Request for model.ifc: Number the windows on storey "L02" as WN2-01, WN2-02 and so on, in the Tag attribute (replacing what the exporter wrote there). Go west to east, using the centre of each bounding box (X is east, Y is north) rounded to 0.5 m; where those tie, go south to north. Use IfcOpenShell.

First a look at what the model holds.

```python
import ifcopenshell
import ifcopenshell.util.element
import ifcopenshell.util.placement

model = ifcopenshell.open("model.ifc")
print(model.schema)
storey = next(s for s in model.by_type("IfcBuildingStorey") if s.Name == "L02")
windows = [e for e in ifcopenshell.util.element.get_decomposition(storey) if e.is_a("IfcWindow")]
for e in sorted(windows, key=lambda e: e.id()):
    origin = ifcopenshell.util.placement.get_local_placement(e.ObjectPlacement)[:3, 3]
    print(e.id(), e.Tag, e.Name, origin.round(2) + 0.0, sep=" | ")
```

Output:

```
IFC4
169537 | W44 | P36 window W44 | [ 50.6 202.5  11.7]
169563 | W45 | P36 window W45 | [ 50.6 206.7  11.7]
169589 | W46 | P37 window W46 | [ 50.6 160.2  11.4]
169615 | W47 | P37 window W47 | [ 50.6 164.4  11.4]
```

```python
import ifcopenshell
import ifcopenshell.geom
import ifcopenshell.util.element
import ifcopenshell.util.shape

model = ifcopenshell.open("model.ifc")
settings = ifcopenshell.geom.settings()
settings.set("use-world-coords", True)


def centre(element):
    shape = ifcopenshell.geom.create_shape(settings, element)
    return ifcopenshell.util.shape.get_bbox_centroid(shape.geometry)


storey = next(s for s in model.by_type("IfcBuildingStorey") if s.Name == "L02")
windows = [e for e in ifcopenshell.util.element.get_decomposition(storey) if e.is_a("IfcWindow")]

# Insertion points can sit at a corner or the storey origin, so sort by the geometry (in metres).
centres = {e: centre(e) for e in windows}
windows.sort(key=lambda e: (round(centres[e][0] / 0.5), centres[e][1]))

for i, e in enumerate(windows, start=1):
    number = f"WN2-{i:02d}"
    e.Tag = number
    print(e.id(), number)

model.write("model_rev.ifc")
```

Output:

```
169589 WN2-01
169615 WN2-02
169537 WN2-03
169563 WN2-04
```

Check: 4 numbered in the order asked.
